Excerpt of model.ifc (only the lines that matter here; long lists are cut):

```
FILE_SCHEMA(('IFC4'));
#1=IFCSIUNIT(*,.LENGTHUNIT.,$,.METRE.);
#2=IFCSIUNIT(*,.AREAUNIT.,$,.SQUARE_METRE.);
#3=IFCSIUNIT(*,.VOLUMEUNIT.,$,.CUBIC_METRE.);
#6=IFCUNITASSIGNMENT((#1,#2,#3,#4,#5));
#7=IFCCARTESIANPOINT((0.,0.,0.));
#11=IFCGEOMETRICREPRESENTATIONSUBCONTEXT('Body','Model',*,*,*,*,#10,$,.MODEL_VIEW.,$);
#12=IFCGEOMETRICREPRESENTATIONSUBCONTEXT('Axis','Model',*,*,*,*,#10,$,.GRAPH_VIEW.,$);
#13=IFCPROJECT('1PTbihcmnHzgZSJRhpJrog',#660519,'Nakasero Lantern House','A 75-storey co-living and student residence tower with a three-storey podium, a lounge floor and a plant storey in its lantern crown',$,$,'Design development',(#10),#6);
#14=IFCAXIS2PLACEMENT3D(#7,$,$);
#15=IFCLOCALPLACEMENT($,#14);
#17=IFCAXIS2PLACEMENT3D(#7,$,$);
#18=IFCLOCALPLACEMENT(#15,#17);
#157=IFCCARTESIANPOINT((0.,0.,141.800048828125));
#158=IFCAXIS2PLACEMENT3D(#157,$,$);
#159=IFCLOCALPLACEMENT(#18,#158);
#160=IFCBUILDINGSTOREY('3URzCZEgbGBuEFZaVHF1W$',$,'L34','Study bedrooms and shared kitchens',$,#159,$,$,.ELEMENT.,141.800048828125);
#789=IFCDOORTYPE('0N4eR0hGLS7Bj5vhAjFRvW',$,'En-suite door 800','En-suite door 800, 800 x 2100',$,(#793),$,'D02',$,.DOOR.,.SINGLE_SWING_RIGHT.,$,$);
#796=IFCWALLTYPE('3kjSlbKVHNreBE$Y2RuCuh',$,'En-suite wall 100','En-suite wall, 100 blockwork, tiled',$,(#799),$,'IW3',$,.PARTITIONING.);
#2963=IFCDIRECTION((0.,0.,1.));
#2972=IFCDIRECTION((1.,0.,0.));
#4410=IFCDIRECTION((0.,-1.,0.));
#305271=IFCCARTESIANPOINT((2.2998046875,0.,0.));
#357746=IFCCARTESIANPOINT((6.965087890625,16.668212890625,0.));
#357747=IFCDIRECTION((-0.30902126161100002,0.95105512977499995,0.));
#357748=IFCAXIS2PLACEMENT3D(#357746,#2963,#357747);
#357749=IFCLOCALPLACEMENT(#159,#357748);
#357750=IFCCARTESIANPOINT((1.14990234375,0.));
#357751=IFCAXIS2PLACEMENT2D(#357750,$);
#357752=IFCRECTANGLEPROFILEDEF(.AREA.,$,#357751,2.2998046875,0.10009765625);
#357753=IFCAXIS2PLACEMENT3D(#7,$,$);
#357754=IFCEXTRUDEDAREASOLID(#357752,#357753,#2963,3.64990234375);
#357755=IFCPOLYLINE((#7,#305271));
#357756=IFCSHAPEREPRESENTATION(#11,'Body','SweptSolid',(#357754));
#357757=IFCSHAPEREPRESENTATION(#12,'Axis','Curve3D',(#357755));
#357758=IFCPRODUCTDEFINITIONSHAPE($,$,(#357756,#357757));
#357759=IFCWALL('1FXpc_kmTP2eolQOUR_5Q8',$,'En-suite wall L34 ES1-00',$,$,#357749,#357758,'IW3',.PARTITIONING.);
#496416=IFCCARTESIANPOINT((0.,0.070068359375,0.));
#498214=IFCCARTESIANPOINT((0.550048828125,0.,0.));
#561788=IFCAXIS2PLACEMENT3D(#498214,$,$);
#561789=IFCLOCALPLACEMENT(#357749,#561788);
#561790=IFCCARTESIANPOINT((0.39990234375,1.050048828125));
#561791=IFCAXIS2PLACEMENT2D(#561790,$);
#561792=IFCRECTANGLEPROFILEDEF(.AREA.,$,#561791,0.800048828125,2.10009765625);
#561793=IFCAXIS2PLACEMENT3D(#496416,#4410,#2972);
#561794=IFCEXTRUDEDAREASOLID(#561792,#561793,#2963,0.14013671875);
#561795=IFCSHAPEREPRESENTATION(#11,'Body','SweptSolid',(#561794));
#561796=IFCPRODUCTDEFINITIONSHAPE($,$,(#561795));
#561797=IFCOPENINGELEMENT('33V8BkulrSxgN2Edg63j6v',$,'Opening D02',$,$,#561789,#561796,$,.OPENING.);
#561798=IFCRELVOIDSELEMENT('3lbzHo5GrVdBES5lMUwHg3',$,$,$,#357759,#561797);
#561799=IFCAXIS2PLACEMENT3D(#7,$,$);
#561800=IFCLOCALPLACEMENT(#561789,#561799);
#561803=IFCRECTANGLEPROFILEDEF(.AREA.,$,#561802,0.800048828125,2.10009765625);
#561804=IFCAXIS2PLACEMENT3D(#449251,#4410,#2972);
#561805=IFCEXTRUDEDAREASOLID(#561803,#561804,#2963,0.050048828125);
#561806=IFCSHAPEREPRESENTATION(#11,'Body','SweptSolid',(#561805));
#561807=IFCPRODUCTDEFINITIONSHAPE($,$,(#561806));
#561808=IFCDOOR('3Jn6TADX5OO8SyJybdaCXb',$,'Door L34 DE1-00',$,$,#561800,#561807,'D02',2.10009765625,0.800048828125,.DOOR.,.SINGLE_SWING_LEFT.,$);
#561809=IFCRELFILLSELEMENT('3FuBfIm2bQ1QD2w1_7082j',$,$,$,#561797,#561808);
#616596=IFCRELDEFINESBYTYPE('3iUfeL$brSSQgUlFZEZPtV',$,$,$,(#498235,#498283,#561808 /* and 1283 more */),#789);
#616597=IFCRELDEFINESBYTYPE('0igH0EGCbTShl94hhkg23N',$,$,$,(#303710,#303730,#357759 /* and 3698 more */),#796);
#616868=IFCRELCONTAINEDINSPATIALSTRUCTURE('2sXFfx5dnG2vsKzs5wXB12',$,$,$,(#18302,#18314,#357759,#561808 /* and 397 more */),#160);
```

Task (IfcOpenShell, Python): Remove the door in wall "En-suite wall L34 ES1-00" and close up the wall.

```python
import ifcopenshell
import ifcopenshell.api.feature
import ifcopenshell.api.root
import ifcopenshell.geom
import ifcopenshell.util.shape

model = ifcopenshell.open("model.ifc")
settings = ifcopenshell.geom.settings()


def volume(element):
    """Net volume in cubic metres, openings subtracted."""
    shape = ifcopenshell.geom.create_shape(settings, element)
    return ifcopenshell.util.shape.get_volume(shape.geometry)


door = model.by_id(561808)
opening = door.FillsVoids[0].RelatingOpeningElement
wall = opening.VoidsElements[0].RelatingBuildingElement
before = volume(wall)

ifcopenshell.api.root.remove_product(model, product=door)
ifcopenshell.api.feature.remove_feature(model, feature=opening)

after = volume(wall)

print(f"wall volume {before:.3f} -> {after:.3f} m3")

model.write("model_rev.ifc")
```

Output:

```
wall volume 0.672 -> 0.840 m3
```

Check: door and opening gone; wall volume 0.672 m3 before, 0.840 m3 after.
